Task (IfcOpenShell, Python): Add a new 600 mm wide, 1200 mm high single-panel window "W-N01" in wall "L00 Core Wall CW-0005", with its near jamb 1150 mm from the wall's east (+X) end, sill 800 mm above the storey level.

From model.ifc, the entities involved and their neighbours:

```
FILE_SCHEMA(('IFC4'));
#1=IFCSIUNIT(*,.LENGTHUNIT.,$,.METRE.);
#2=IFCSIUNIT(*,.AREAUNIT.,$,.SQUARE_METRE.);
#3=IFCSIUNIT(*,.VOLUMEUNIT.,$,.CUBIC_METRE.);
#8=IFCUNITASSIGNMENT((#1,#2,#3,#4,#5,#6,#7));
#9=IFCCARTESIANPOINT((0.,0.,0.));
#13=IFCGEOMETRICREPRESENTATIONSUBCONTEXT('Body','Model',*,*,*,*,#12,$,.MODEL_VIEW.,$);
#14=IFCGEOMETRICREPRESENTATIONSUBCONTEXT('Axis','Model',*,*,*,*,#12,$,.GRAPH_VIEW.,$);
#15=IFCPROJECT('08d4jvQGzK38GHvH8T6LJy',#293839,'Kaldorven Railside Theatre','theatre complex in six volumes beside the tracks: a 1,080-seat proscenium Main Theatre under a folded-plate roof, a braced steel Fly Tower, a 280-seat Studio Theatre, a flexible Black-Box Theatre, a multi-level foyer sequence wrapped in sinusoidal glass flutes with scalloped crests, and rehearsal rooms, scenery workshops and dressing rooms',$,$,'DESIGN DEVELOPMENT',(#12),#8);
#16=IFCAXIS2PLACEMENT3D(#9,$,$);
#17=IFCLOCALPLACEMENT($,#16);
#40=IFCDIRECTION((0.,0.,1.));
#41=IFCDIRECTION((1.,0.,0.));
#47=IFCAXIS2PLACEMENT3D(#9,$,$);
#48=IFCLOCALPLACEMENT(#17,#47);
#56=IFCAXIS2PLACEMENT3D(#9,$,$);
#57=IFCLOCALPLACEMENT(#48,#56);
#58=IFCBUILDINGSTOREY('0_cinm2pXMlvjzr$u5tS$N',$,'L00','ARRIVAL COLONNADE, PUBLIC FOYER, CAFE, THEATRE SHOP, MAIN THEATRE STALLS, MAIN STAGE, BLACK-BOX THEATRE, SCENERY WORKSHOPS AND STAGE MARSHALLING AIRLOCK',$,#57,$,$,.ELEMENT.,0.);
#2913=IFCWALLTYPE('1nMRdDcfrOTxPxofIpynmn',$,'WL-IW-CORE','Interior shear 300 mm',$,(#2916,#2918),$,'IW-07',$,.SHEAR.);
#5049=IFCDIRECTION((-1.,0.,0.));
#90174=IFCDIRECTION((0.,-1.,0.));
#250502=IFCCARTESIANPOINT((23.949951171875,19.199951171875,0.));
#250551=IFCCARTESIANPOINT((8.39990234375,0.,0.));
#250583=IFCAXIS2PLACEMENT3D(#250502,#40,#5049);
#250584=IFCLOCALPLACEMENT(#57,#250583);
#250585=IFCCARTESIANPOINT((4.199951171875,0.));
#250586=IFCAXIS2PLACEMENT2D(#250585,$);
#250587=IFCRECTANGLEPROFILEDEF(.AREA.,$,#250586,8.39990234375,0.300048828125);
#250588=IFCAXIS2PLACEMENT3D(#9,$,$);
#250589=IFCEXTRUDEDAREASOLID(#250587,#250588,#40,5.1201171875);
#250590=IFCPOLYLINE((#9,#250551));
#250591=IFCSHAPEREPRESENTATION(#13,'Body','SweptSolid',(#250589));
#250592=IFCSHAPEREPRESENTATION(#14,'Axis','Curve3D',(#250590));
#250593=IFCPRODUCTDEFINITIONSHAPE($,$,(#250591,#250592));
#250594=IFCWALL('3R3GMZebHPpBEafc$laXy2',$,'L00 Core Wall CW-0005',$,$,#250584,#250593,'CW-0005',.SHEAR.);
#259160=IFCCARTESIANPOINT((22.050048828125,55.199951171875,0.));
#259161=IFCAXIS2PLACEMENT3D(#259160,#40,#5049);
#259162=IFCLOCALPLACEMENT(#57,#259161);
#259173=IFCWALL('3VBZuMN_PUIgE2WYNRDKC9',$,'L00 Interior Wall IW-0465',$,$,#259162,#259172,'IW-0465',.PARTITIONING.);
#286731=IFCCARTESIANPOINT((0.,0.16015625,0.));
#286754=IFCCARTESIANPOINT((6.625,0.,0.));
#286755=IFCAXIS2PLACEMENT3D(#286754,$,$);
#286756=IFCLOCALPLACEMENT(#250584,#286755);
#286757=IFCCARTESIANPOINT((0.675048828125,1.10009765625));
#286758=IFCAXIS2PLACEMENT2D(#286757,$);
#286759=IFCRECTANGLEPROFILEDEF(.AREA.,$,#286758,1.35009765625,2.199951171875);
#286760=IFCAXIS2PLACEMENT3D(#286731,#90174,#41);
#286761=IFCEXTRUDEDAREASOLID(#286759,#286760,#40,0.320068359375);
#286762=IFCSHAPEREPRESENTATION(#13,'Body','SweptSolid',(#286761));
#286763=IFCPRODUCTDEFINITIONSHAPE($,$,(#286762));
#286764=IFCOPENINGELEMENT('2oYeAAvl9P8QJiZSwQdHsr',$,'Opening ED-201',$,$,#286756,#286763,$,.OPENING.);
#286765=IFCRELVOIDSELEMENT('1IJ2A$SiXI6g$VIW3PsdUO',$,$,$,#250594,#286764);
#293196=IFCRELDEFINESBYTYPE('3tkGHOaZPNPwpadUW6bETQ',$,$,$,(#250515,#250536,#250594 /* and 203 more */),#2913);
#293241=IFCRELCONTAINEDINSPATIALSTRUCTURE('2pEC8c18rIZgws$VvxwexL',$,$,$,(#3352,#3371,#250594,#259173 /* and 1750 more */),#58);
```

```python
import numpy as np
import ifcopenshell
import ifcopenshell.api.feature
import ifcopenshell.api.geometry
import ifcopenshell.api.root
import ifcopenshell.api.spatial
import ifcopenshell.geom
import ifcopenshell.util.element
import ifcopenshell.util.placement
import ifcopenshell.util.representation
import ifcopenshell.util.shape
import ifcopenshell.util.unit

model = ifcopenshell.open("model.ifc")
unit_scale = ifcopenshell.util.unit.calculate_unit_scale(model)
settings = ifcopenshell.geom.settings()


def volume(element):
    """Net volume in cubic metres, openings subtracted."""
    shape = ifcopenshell.geom.create_shape(settings, element)
    return ifcopenshell.util.shape.get_volume(shape.geometry)


wall = model.by_guid("3R3GMZebHPpBEafc$laXy2")
storey = ifcopenshell.util.element.get_container(wall, ifc_class="IfcBuildingStorey")
context = ifcopenshell.util.representation.get_context(model, "Model", "Body", "MODEL_VIEW")
before = volume(wall)

width, height, from_end, sill = 0.6, 1.2, 1.15, 0.8  # metres

# The wall runs along its own X axis, and the end named is its -X end.
wall_shape = ifcopenshell.geom.create_shape(settings, wall)
x, y, z = ifcopenshell.util.shape.get_vertices(wall_shape.geometry).T
start = x.min() + from_end
face, thickness = float(y.min()), float(y.max() - y.min())
wall_matrix = ifcopenshell.util.placement.get_local_placement(wall.ObjectPlacement)
level = ifcopenshell.util.placement.get_local_placement(storey.ObjectPlacement)[2, 3]


def in_wall(x, y):
    """Placement at x, y metres in the wall's axes, at sill height."""
    matrix = wall_matrix.copy()
    matrix[:, 3] = wall_matrix @ np.array([x / unit_scale, y / unit_scale, 0.0, 1.0])
    matrix[2, 3] = level + sill / unit_scale
    return matrix


# Opening: a box that overshoots both wall faces by 50 mm.
opening = ifcopenshell.api.root.create_entity(model, ifc_class="IfcOpeningElement", predefined_type="OPENING")
box = ifcopenshell.api.geometry.add_wall_representation(
    model, context=context, length=width, height=height, thickness=thickness + 0.1
)
ifcopenshell.api.geometry.assign_representation(model, product=opening, representation=box)
ifcopenshell.api.geometry.edit_object_placement(model, product=opening, matrix=in_wall(start, face - 0.05), is_si=False)
ifcopenshell.api.feature.add_feature(model, feature=opening, element=wall)

window = ifcopenshell.api.root.create_entity(model, ifc_class="IfcWindow", name="W-N01", predefined_type="WINDOW")
window.OverallWidth, window.OverallHeight = width / unit_scale, height / unit_scale
window.PartitioningType = "SINGLE_PANEL"
body = ifcopenshell.api.geometry.add_window_representation(
    model,
    context=context,
    overall_width=window.OverallWidth,
    overall_height=window.OverallHeight,
    partition_type="SINGLE_PANEL",
)
ifcopenshell.api.geometry.assign_representation(model, product=window, representation=body)
ifcopenshell.api.spatial.assign_container(model, products=[window], relating_structure=storey)
ifcopenshell.api.feature.add_filling(model, opening=opening, element=window)

# Centre the window in the wall's thickness.
ifcopenshell.api.geometry.edit_object_placement(model, product=window, matrix=in_wall(start, face), is_si=False)
window_shape = ifcopenshell.geom.create_shape(settings, window)
depth = ifcopenshell.util.shape.get_vertices(window_shape.geometry)[:, 1]
offset = face + thickness / 2 - (depth.min() + depth.max()) / 2
ifcopenshell.api.geometry.edit_object_placement(model, product=window, matrix=in_wall(start, offset), is_si=False)

after = volume(wall)

print(f"wall volume {before:.3f} -> {after:.3f} m3")

model.write("model_updated.ifc")
```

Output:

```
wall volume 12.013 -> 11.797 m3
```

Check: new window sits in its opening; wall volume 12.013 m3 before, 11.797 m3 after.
